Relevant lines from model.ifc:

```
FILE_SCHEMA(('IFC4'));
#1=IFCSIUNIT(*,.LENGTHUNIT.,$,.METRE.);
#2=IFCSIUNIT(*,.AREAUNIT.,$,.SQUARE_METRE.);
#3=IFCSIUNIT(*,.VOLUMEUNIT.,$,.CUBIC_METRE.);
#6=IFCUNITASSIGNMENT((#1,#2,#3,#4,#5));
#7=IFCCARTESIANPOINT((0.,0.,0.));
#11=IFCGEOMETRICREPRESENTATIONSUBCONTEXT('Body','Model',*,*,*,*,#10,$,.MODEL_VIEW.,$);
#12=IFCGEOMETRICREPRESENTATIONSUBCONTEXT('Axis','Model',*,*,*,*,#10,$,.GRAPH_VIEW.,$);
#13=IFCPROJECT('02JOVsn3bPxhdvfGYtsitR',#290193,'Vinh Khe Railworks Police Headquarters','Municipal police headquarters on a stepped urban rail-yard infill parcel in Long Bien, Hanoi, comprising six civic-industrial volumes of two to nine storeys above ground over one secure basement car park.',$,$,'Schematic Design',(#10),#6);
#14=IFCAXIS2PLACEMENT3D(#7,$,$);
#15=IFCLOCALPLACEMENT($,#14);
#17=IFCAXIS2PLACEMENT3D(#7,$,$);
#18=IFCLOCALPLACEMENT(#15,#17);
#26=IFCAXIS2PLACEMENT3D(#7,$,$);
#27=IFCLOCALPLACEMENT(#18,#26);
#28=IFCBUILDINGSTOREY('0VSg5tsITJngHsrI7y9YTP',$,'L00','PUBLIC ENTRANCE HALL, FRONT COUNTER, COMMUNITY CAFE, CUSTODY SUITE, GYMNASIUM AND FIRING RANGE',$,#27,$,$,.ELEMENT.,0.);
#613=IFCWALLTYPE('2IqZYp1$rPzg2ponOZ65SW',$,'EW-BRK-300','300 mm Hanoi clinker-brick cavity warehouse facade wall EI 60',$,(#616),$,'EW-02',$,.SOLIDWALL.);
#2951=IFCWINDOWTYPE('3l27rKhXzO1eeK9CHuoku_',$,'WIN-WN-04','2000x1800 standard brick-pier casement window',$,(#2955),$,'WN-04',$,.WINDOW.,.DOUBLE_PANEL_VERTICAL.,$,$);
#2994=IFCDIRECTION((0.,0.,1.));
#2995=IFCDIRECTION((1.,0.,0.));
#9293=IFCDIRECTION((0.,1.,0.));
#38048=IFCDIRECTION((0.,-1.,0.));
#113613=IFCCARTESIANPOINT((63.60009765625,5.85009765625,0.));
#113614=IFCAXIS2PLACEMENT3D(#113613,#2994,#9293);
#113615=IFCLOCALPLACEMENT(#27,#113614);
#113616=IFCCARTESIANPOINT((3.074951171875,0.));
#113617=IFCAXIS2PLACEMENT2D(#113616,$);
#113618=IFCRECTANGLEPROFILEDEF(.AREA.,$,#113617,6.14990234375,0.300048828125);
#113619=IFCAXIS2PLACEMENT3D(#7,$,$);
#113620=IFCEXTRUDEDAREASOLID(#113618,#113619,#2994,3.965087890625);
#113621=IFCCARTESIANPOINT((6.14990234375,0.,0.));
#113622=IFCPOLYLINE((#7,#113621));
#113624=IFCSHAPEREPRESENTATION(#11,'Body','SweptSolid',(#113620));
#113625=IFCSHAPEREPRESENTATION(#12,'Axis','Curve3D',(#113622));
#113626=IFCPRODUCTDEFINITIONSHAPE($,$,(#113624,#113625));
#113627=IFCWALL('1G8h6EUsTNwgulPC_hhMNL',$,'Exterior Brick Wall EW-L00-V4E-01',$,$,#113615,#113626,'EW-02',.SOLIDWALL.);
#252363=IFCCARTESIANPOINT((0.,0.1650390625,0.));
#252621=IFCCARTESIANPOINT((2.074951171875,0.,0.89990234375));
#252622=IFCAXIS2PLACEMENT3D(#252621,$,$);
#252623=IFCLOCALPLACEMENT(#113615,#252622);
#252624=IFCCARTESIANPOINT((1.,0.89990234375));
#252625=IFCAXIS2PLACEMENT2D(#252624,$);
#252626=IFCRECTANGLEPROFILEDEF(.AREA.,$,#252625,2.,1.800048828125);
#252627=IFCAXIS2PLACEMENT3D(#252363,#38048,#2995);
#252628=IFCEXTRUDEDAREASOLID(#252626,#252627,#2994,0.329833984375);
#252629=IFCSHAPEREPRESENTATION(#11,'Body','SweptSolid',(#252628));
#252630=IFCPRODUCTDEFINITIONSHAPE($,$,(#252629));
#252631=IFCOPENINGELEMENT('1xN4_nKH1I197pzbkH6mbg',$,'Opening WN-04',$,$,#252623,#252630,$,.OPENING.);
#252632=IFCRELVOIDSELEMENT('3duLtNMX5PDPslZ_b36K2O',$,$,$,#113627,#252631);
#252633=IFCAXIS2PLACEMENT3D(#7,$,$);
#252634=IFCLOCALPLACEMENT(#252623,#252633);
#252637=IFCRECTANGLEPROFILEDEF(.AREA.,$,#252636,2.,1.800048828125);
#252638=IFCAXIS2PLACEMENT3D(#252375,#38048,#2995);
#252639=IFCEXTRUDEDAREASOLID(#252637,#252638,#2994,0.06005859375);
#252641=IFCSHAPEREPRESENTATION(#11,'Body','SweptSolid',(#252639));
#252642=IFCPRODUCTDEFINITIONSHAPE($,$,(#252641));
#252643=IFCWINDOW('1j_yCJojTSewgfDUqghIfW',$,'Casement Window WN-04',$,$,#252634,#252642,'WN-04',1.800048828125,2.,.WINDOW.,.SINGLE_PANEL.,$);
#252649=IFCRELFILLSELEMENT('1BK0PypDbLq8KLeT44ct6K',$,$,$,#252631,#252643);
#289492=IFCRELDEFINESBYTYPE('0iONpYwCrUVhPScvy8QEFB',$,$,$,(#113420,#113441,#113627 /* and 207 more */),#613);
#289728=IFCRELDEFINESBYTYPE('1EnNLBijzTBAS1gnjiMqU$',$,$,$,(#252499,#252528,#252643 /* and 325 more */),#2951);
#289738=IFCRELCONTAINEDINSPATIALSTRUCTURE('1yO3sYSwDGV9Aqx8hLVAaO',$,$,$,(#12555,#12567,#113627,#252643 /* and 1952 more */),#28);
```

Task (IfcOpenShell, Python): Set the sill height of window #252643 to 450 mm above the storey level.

```python
import numpy as np
import ifcopenshell
import ifcopenshell.api.geometry
import ifcopenshell.geom
import ifcopenshell.util.element
import ifcopenshell.util.placement
import ifcopenshell.util.shape
import ifcopenshell.util.unit

model = ifcopenshell.open("model.ifc")
unit_scale = ifcopenshell.util.unit.calculate_unit_scale(model)

window = model.by_id(252643)
opening = window.FillsVoids[0].RelatingOpeningElement
storey = ifcopenshell.util.element.get_container(window, ifc_class="IfcBuildingStorey")
level = ifcopenshell.util.placement.get_local_placement(storey.ObjectPlacement)[2, 3]

# The opening's origin need not be at the sill, so measure its lowest point.
shape = ifcopenshell.geom.create_shape(ifcopenshell.geom.settings(), opening)
bottom = ifcopenshell.util.shape.get_shape_bottom_elevation(shape, shape.geometry) / unit_scale
dz = level + 0.45 - bottom

shift = np.array([0.0, 0.0, dz])
# The window is placed relative to its opening, so it follows when the opening moves.
matrix = ifcopenshell.util.placement.get_local_placement(opening.ObjectPlacement)
matrix[:3, 3] += shift
ifcopenshell.api.geometry.edit_object_placement(
    model, product=opening, matrix=matrix, is_si=False, should_transform_children=True
)

print(f"moved by {dz * unit_scale:+.3f} m")

model.write("model_v2.ifc")
```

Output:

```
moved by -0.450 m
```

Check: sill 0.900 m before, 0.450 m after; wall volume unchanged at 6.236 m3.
